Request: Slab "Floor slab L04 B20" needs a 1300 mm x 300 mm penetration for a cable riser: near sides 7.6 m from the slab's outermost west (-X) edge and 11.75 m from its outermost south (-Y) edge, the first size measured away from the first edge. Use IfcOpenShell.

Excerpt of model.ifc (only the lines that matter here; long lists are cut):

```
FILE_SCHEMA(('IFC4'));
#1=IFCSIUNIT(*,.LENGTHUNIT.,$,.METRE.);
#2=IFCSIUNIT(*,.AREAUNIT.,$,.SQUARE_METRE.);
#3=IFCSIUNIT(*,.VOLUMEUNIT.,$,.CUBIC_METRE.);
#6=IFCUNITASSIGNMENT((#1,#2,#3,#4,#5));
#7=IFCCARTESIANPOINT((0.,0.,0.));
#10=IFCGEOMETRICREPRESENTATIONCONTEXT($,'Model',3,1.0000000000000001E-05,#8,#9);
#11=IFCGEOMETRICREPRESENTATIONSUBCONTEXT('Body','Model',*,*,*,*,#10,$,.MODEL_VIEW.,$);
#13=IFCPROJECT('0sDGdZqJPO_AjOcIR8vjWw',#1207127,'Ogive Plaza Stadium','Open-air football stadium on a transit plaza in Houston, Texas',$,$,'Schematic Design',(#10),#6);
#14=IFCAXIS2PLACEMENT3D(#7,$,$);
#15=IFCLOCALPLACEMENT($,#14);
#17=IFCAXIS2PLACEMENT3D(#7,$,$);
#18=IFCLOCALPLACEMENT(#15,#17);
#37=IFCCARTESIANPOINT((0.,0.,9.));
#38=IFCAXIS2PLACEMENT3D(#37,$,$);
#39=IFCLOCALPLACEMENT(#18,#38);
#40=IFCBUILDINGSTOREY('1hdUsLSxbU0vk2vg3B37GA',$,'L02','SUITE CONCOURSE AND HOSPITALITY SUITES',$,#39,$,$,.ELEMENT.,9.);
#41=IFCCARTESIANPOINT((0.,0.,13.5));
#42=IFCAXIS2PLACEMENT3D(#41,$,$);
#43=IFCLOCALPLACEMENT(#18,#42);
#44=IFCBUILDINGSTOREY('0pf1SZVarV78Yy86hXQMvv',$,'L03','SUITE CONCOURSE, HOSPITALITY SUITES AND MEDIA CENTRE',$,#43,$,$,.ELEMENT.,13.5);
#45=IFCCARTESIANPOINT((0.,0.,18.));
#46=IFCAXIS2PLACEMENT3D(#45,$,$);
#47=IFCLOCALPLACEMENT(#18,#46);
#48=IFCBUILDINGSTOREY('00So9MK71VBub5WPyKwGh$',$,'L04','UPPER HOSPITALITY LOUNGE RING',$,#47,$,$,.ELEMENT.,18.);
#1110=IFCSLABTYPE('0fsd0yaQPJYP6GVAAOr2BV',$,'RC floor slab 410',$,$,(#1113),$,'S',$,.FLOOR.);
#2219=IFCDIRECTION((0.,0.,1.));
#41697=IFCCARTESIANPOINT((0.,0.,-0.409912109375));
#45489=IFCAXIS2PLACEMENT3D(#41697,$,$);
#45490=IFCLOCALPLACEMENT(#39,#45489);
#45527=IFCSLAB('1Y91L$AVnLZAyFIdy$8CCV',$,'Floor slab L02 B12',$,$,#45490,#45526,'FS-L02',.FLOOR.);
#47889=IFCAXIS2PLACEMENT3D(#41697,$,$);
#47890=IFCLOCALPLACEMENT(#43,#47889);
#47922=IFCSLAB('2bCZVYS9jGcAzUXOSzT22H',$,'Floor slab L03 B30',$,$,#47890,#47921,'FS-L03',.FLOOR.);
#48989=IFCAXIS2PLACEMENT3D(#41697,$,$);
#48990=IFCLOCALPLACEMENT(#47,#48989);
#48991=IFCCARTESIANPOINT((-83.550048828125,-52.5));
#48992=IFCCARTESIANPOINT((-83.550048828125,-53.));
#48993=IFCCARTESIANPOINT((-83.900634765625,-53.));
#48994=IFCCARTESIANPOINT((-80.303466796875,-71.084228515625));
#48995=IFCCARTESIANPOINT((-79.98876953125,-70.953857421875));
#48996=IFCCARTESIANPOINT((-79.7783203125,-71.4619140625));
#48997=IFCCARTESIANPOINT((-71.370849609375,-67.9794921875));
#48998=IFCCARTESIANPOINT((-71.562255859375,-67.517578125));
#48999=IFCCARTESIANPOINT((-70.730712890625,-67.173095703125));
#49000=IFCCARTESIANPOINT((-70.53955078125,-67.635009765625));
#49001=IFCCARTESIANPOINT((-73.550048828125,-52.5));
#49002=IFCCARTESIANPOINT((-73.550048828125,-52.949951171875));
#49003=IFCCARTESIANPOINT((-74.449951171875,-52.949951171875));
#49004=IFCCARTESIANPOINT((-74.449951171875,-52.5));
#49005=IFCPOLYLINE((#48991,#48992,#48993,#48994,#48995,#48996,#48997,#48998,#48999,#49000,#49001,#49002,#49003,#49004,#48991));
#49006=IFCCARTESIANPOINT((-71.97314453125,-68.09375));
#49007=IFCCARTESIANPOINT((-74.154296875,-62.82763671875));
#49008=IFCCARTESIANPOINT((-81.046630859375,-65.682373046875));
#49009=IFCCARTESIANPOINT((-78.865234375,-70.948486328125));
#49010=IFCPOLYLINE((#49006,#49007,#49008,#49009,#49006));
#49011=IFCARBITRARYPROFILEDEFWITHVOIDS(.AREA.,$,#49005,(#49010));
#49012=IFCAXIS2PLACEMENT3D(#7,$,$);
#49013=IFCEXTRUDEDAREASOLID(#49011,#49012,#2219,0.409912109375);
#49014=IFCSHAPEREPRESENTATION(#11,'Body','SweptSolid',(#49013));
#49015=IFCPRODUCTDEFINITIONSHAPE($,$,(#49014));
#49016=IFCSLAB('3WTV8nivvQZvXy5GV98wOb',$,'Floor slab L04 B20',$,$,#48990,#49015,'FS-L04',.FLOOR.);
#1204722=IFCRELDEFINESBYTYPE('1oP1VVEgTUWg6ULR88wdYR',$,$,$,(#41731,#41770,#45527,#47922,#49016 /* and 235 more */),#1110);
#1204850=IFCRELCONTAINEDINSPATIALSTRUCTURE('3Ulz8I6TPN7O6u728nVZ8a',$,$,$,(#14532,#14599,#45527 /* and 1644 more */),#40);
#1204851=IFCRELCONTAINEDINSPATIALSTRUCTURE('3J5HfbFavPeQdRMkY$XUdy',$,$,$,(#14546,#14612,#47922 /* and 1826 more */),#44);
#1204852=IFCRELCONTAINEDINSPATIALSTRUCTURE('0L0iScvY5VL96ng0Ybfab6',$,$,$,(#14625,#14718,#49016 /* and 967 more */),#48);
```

```python
import numpy as np
import ifcopenshell
import ifcopenshell.api.feature
import ifcopenshell.api.geometry
import ifcopenshell.api.root
import ifcopenshell.geom
import ifcopenshell.util.placement
import ifcopenshell.util.representation
import ifcopenshell.util.shape
import ifcopenshell.util.unit

model = ifcopenshell.open("model.ifc")
unit_scale = ifcopenshell.util.unit.calculate_unit_scale(model)
settings = ifcopenshell.geom.settings()


def volume(element):
    """Net volume in cubic metres, openings subtracted."""
    shape = ifcopenshell.geom.create_shape(settings, element)
    return ifcopenshell.util.shape.get_volume(shape.geometry)


slab = model.by_guid("3WTV8nivvQZvXy5GV98wOb")
before = volume(slab)

# Extent in the slab's own axes, in metres. The edges named are its -X and -Y sides.
slab_shape = ifcopenshell.geom.create_shape(settings, slab)
vertices = ifcopenshell.util.shape.get_vertices(slab_shape.geometry)
x_min, y_min, bottom = vertices.min(axis=0)
top = vertices[:, 2].max()

opening = ifcopenshell.api.root.create_entity(model, ifc_class="IfcOpeningElement", name="Cable riser opening", predefined_type="OPENING")
context = ifcopenshell.util.representation.get_context(model, "Model", "Body", "MODEL_VIEW")
width, depth = 1.3, 0.3
outline = [(0.0, 0.0), (width, 0.0), (width, depth), (0.0, depth), (0.0, 0.0)]
# Overshoot both faces by 50 mm so the cut is clean.
shape = ifcopenshell.api.geometry.add_slab_representation(
    model, context=context, depth=top - bottom + 0.1, polyline=outline
)
ifcopenshell.api.geometry.assign_representation(model, product=opening, representation=shape)

matrix = ifcopenshell.util.placement.get_local_placement(slab.ObjectPlacement)
matrix[:, 3] = matrix @ np.append(np.array([x_min + 7.6, y_min + 11.75, bottom - 0.05]) / unit_scale, 1.0)
ifcopenshell.api.geometry.edit_object_placement(model, product=opening, matrix=matrix, is_si=False)
ifcopenshell.api.feature.add_feature(model, feature=opening, element=slab)

after = volume(slab)

print(f"slab volume {before:.3f} -> {after:.3f} m3")

model.write("model_rev.ifc")
```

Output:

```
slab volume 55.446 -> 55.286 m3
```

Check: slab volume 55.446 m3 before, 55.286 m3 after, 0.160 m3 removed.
